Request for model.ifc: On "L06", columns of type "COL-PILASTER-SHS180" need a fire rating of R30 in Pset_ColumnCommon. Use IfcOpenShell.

First a look at what the model holds.

```python
import ifcopenshell
import ifcopenshell.util.element

model = ifcopenshell.open("model.ifc")
print(model.schema)
storey = next(s for s in model.by_type("IfcBuildingStorey") if s.Name == "L06")
columns = [e for e in ifcopenshell.util.element.get_decomposition(storey) if e.is_a("IfcColumn")]
seen = {}
for e in columns:
    element_type = ifcopenshell.util.element.get_type(e)
    key = (element_type.Name if element_type != e and element_type else None, ifcopenshell.util.element.get_pset(e, "Pset_ColumnCommon", "FireRating"))
    seen[key] = seen.get(key, 0) + 1
for (name, value), count in sorted(seen.items(), key=str):
    print(count, "x", name, "|", value)
```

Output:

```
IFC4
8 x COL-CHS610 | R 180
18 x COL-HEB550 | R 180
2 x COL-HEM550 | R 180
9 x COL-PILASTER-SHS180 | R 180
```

```python
import ifcopenshell
import ifcopenshell.api.pset
import ifcopenshell.util.element

model = ifcopenshell.open("model.ifc")

storey = next(s for s in model.by_type("IfcBuildingStorey") if s.Name == "L06")
columns = [e for e in ifcopenshell.util.element.get_decomposition(storey) if e.is_a("IfcColumn")]

count = 0
for e in columns:
    element_type = ifcopenshell.util.element.get_type(e)
    if element_type in (None, e) or element_type.Name != "COL-PILASTER-SHS180":
        continue
    # add_pset returns the element's existing set when there is one.
    pset = ifcopenshell.api.pset.add_pset(model, product=e, name="Pset_ColumnCommon")
    ifcopenshell.api.pset.edit_pset(model, pset=pset, properties={"FireRating": "R30"})
    count += 1

print(count, "columns updated")

model.write("model-out.ifc")
```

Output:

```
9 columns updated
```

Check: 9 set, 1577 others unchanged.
